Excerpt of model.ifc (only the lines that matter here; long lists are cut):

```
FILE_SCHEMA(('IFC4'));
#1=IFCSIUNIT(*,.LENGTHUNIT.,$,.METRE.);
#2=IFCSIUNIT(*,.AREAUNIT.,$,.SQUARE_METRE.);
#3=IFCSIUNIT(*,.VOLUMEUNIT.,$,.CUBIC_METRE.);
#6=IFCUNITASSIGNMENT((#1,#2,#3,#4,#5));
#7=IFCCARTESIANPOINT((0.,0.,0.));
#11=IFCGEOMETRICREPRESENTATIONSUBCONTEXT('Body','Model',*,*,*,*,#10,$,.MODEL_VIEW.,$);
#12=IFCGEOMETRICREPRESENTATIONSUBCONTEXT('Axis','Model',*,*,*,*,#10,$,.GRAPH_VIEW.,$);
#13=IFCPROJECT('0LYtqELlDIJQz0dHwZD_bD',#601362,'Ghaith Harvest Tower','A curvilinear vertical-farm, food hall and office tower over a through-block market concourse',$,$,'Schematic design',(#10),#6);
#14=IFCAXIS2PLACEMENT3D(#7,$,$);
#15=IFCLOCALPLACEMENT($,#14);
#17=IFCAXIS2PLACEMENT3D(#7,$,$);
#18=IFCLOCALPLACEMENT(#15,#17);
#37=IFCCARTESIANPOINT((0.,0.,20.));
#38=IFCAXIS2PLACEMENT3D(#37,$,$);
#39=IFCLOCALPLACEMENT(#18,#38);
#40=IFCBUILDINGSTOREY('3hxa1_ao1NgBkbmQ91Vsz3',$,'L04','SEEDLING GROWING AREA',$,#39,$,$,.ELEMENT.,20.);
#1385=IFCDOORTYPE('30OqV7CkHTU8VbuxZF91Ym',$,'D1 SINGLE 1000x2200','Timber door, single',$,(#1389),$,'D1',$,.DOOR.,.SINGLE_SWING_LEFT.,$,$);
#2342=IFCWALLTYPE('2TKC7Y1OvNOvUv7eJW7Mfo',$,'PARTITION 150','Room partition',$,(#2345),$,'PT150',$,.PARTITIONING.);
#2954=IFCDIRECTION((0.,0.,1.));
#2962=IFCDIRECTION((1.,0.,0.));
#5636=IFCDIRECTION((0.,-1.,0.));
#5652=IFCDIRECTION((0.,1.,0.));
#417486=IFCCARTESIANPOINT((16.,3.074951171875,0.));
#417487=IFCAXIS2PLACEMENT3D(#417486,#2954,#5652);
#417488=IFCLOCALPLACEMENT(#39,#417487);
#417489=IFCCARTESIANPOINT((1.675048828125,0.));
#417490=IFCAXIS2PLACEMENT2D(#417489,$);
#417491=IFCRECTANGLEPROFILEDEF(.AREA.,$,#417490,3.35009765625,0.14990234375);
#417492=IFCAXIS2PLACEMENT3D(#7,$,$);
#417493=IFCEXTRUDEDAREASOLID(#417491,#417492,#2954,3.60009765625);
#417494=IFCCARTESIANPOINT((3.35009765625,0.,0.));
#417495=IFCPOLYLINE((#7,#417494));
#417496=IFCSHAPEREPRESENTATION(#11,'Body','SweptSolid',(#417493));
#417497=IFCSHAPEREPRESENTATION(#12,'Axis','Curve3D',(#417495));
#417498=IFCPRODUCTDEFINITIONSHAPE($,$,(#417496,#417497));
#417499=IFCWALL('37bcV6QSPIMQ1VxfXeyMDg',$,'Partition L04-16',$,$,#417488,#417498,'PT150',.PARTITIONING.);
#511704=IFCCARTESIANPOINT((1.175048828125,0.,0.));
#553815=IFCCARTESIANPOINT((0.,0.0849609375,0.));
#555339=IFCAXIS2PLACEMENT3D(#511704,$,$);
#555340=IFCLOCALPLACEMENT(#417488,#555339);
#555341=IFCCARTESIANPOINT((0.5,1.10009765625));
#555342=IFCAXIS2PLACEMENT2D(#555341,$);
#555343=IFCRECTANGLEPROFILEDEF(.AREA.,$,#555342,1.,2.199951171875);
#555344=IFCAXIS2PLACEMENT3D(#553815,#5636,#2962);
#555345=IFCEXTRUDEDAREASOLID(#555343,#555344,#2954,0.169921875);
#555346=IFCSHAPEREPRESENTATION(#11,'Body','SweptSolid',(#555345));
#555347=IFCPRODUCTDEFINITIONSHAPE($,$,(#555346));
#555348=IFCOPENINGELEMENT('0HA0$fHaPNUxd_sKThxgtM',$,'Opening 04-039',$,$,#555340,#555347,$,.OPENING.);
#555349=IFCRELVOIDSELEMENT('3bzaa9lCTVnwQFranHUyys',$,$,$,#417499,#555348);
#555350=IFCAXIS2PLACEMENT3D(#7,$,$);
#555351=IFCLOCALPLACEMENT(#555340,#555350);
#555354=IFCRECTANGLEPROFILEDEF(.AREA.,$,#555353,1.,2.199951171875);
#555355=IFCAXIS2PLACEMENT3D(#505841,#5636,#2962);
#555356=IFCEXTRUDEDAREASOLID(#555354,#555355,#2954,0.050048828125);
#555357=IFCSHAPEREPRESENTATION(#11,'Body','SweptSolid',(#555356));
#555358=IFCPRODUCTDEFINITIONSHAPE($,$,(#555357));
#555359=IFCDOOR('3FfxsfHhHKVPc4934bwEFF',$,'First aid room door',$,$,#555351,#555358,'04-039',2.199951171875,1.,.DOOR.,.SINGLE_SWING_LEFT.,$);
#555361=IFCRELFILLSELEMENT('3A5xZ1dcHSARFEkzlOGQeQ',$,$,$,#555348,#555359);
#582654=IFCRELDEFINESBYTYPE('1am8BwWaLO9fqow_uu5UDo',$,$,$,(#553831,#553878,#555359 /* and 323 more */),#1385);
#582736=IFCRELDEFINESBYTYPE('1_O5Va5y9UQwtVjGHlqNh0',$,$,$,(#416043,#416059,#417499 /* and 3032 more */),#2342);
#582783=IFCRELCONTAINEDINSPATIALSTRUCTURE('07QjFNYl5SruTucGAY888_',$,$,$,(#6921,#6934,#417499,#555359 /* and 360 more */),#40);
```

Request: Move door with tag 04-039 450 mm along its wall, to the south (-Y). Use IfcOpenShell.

```python
import ifcopenshell
import ifcopenshell.api.geometry
import ifcopenshell.util.placement

model = ifcopenshell.open("model.ifc")

door = model.by_guid("3FfxsfHhHKVPc4934bwEFF")
opening = door.FillsVoids[0].RelatingOpeningElement
wall = opening.VoidsElements[0].RelatingBuildingElement

wall_matrix = ifcopenshell.util.placement.get_local_placement(wall.ObjectPlacement)
shift = wall_matrix[:3, 0] * -0.45
before = ifcopenshell.util.placement.get_local_placement(door.ObjectPlacement)[:3, 3].copy()

# The door is placed relative to its opening, so it follows when the opening moves.
matrix = ifcopenshell.util.placement.get_local_placement(opening.ObjectPlacement)
matrix[:3, 3] += shift
ifcopenshell.api.geometry.edit_object_placement(
    model, product=opening, matrix=matrix, is_si=False, should_transform_children=True
)

after = ifcopenshell.util.placement.get_local_placement(door.ObjectPlacement)[:3, 3]
print("door moved by", (after - before).round(3) + 0.0)

model.write("model_updated.ifc")
```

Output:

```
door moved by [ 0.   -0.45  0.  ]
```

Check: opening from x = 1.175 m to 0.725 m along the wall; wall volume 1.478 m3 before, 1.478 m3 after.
